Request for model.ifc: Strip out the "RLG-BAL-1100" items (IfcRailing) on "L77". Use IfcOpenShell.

First a look at what the model holds.

```python
import ifcopenshell
import ifcopenshell.util.element

model = ifcopenshell.open("model.ifc")
print(model.schema)
storey = next(s for s in model.by_type("IfcBuildingStorey") if s.Name == "L77")
railings = [e for e in ifcopenshell.util.element.get_decomposition(storey) if e.is_a("IfcRailing")]
seen = {}
for e in railings:
    element_type = ifcopenshell.util.element.get_type(e)
    name = element_type.Name if element_type not in (None, e) else None
    seen[name] = seen.get(name, 0) + 1
for name, count in sorted(seen.items(), key=str):
    print(count, "x", name)
```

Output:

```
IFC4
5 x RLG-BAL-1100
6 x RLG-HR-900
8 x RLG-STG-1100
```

```python
import ifcopenshell
import ifcopenshell.api.root
import ifcopenshell.util.element

model = ifcopenshell.open("model.ifc")

storey = next(s for s in model.by_type("IfcBuildingStorey") if s.Name == "L77")
railings = [e for e in ifcopenshell.util.element.get_decomposition(storey) if e.is_a("IfcRailing")]
targets = [e for e in railings if (t := ifcopenshell.util.element.get_type(e)) not in (None, e) and t.Name == "RLG-BAL-1100"]

for e in targets:
    ifcopenshell.api.root.remove_product(model, product=e)
print(len(targets), "removed")

model.write("model_v2.ifc")
```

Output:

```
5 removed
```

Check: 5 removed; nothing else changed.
